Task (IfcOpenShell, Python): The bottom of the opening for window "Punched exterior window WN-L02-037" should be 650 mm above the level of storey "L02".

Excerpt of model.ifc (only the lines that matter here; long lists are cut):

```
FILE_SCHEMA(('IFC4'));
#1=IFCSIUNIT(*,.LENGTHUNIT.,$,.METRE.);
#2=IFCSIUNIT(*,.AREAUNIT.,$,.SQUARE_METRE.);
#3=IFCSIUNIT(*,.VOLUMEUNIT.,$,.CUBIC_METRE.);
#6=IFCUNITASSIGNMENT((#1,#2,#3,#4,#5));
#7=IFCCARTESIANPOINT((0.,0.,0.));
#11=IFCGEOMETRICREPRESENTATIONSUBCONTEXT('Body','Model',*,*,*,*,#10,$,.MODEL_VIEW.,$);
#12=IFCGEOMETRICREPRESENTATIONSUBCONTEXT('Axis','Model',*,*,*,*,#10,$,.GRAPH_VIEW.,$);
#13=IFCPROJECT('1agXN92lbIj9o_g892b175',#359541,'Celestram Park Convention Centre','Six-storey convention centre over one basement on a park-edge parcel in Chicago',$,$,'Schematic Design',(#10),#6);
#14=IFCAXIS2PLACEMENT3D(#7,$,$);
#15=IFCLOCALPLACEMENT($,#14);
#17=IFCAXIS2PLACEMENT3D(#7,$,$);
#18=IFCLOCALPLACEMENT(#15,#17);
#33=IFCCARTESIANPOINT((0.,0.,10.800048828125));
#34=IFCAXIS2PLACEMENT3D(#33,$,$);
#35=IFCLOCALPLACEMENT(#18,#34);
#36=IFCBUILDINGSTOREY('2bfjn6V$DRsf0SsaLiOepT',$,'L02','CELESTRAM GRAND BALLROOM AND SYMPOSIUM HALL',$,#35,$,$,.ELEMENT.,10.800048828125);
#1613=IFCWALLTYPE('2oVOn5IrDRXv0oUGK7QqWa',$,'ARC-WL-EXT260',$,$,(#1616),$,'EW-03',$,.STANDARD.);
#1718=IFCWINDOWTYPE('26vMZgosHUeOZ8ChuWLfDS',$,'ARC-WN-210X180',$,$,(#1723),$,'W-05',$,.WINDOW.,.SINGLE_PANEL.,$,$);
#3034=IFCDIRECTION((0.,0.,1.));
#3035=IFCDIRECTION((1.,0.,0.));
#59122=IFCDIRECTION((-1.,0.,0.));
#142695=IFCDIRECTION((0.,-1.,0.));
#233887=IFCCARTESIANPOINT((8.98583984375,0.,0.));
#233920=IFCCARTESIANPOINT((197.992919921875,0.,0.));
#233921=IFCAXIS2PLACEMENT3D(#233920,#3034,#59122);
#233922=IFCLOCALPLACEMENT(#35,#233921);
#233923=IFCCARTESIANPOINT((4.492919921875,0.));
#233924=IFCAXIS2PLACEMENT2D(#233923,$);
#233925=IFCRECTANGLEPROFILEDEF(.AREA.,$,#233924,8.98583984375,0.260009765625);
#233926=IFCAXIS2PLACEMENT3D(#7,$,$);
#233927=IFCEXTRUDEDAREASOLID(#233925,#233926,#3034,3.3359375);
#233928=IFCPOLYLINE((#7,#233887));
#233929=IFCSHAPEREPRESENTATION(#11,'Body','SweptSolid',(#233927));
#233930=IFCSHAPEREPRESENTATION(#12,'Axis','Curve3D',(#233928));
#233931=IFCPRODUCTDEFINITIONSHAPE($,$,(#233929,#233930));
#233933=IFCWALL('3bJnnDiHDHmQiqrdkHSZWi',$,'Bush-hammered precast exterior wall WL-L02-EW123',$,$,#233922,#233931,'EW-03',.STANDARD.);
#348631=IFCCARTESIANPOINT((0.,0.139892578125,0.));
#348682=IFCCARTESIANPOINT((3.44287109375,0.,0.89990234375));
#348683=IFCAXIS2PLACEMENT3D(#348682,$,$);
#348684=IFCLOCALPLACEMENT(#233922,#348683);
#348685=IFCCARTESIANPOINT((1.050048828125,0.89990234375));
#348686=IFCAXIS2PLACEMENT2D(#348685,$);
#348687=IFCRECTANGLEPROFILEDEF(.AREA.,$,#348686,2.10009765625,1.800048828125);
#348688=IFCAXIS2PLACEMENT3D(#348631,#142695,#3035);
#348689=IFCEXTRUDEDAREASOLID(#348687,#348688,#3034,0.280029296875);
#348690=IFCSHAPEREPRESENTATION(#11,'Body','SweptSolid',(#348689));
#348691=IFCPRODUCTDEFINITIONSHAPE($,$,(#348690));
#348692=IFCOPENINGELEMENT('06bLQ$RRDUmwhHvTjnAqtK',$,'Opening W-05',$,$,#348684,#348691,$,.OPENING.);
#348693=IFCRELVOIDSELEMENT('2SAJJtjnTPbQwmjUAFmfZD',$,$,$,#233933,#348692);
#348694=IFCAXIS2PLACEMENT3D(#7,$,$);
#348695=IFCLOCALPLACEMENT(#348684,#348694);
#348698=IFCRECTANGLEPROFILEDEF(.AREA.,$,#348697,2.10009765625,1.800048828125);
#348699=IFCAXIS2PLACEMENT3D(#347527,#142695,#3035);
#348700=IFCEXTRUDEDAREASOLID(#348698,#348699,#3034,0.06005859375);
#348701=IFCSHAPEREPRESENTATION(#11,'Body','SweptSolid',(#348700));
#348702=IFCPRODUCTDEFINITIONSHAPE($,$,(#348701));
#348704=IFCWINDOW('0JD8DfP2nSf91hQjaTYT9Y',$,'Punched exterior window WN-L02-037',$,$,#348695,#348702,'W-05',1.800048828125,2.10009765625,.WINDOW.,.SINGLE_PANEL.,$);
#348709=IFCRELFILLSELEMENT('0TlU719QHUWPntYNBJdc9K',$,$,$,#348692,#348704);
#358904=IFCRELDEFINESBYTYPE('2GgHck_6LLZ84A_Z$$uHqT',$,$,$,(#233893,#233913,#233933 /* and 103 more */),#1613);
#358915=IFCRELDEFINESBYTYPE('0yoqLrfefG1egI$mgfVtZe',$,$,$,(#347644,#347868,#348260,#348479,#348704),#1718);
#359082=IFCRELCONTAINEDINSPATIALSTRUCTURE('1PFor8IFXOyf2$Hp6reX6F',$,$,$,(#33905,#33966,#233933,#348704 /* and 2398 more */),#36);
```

```python
import numpy as np
import ifcopenshell
import ifcopenshell.api.geometry
import ifcopenshell.geom
import ifcopenshell.util.element
import ifcopenshell.util.placement
import ifcopenshell.util.shape
import ifcopenshell.util.unit

model = ifcopenshell.open("model.ifc")
unit_scale = ifcopenshell.util.unit.calculate_unit_scale(model)

window = model.by_id(348704)
opening = window.FillsVoids[0].RelatingOpeningElement
storey = ifcopenshell.util.element.get_container(window, ifc_class="IfcBuildingStorey")
level = ifcopenshell.util.placement.get_local_placement(storey.ObjectPlacement)[2, 3]

# The opening's origin need not be at the sill, so measure its lowest point.
shape = ifcopenshell.geom.create_shape(ifcopenshell.geom.settings(), opening)
bottom = ifcopenshell.util.shape.get_shape_bottom_elevation(shape, shape.geometry) / unit_scale
dz = level + 0.65 / unit_scale - bottom

shift = np.array([0.0, 0.0, dz])
# The window is placed relative to its opening, so it follows when the opening moves.
matrix = ifcopenshell.util.placement.get_local_placement(opening.ObjectPlacement)
matrix[:3, 3] += shift
ifcopenshell.api.geometry.edit_object_placement(
    model, product=opening, matrix=matrix, is_si=False, should_transform_children=True
)

print(f"moved by {dz * unit_scale:+.3f} m")

model.write("model_v2.ifc")
```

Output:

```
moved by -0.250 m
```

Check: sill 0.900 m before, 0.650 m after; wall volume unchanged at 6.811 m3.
